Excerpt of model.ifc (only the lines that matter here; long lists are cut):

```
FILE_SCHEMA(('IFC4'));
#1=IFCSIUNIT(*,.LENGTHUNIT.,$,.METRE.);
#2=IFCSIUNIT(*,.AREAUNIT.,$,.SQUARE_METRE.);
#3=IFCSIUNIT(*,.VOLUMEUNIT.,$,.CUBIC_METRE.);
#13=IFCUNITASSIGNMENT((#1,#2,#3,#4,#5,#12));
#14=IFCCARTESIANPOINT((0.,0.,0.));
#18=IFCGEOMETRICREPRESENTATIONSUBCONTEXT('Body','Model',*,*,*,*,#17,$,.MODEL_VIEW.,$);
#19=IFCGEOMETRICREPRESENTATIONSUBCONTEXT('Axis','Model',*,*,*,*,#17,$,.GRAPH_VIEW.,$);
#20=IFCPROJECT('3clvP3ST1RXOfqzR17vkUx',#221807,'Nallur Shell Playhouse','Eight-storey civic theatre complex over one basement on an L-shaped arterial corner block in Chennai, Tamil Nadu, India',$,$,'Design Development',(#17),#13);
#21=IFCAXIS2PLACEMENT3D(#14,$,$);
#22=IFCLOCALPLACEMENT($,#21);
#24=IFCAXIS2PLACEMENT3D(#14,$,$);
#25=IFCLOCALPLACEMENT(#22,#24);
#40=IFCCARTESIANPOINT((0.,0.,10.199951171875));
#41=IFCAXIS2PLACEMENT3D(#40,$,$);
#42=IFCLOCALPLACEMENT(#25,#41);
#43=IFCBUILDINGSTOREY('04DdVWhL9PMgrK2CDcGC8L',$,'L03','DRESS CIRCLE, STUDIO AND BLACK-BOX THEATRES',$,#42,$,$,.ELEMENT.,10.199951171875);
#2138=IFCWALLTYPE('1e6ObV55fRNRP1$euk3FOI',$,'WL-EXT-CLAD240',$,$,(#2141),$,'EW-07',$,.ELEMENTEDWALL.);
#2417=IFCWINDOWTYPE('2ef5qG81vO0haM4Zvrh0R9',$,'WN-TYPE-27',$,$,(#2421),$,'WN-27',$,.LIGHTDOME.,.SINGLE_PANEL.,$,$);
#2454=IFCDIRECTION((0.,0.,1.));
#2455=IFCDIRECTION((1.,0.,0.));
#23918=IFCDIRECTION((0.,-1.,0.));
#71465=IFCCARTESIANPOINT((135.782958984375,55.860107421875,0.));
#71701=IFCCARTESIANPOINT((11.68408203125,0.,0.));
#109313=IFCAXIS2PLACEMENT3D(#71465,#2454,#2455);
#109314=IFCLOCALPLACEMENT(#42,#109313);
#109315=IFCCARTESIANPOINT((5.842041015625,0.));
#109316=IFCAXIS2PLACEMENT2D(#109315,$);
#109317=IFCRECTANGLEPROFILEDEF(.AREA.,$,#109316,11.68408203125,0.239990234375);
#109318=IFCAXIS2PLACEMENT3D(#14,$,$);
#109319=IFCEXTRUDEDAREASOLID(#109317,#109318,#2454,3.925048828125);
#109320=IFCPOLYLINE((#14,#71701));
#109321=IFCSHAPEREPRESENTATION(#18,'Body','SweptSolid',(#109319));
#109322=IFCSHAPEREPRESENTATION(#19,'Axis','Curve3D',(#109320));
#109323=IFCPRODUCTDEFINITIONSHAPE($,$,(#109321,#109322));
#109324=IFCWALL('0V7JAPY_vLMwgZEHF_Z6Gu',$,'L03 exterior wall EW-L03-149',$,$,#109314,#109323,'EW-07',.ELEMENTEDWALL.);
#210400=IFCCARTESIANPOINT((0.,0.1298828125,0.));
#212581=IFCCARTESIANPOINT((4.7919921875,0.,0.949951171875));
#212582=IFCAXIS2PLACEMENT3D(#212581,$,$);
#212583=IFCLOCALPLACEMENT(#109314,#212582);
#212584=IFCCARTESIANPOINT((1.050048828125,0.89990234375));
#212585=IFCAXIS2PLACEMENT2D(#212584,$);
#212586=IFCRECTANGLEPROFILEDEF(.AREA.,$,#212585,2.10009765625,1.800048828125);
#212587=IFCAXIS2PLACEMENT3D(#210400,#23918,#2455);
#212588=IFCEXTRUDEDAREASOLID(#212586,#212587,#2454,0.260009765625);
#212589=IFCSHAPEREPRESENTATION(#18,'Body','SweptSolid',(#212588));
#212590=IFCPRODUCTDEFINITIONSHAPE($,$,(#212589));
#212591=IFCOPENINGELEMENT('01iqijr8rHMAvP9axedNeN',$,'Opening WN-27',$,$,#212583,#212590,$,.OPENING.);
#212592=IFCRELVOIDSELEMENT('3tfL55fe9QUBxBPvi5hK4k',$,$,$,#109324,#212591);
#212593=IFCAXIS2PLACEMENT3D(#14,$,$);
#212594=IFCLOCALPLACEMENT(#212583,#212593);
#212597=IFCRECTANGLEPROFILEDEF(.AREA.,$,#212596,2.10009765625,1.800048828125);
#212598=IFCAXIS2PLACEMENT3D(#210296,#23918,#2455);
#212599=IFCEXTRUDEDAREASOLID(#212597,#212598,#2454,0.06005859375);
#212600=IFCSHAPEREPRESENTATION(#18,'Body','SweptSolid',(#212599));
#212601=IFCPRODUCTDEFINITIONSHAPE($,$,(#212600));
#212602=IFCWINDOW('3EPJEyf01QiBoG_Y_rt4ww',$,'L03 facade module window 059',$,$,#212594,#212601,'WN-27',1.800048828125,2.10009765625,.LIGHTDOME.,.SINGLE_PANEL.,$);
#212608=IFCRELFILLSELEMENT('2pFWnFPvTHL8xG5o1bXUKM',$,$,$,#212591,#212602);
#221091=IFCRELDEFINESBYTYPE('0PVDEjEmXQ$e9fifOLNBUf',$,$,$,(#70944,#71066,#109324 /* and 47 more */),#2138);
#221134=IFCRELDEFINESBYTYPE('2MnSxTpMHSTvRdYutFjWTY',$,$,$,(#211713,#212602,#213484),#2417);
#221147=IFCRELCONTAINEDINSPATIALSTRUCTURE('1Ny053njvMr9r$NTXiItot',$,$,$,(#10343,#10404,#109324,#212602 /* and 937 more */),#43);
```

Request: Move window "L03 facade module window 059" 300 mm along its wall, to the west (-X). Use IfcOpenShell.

```python
import ifcopenshell
import ifcopenshell.api.geometry
import ifcopenshell.util.placement
import ifcopenshell.util.unit

model = ifcopenshell.open("model.ifc")
unit_scale = ifcopenshell.util.unit.calculate_unit_scale(model)

window = model.by_guid("3EPJEyf01QiBoG_Y_rt4ww")
opening = window.FillsVoids[0].RelatingOpeningElement
wall = opening.VoidsElements[0].RelatingBuildingElement

wall_matrix = ifcopenshell.util.placement.get_local_placement(wall.ObjectPlacement)
shift = wall_matrix[:3, 0] * -0.3 / unit_scale
before = ifcopenshell.util.placement.get_local_placement(window.ObjectPlacement)[:3, 3].copy()

# The window is placed relative to its opening, so it follows when the opening moves.
matrix = ifcopenshell.util.placement.get_local_placement(opening.ObjectPlacement)
matrix[:3, 3] += shift
ifcopenshell.api.geometry.edit_object_placement(
    model, product=opening, matrix=matrix, is_si=False, should_transform_children=True
)

after = ifcopenshell.util.placement.get_local_placement(window.ObjectPlacement)[:3, 3]
print("window moved by", (after - before).round(3) + 0.0)

model.write("model_v2.ifc")
```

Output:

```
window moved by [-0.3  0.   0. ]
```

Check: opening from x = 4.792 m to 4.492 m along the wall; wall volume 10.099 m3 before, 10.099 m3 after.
